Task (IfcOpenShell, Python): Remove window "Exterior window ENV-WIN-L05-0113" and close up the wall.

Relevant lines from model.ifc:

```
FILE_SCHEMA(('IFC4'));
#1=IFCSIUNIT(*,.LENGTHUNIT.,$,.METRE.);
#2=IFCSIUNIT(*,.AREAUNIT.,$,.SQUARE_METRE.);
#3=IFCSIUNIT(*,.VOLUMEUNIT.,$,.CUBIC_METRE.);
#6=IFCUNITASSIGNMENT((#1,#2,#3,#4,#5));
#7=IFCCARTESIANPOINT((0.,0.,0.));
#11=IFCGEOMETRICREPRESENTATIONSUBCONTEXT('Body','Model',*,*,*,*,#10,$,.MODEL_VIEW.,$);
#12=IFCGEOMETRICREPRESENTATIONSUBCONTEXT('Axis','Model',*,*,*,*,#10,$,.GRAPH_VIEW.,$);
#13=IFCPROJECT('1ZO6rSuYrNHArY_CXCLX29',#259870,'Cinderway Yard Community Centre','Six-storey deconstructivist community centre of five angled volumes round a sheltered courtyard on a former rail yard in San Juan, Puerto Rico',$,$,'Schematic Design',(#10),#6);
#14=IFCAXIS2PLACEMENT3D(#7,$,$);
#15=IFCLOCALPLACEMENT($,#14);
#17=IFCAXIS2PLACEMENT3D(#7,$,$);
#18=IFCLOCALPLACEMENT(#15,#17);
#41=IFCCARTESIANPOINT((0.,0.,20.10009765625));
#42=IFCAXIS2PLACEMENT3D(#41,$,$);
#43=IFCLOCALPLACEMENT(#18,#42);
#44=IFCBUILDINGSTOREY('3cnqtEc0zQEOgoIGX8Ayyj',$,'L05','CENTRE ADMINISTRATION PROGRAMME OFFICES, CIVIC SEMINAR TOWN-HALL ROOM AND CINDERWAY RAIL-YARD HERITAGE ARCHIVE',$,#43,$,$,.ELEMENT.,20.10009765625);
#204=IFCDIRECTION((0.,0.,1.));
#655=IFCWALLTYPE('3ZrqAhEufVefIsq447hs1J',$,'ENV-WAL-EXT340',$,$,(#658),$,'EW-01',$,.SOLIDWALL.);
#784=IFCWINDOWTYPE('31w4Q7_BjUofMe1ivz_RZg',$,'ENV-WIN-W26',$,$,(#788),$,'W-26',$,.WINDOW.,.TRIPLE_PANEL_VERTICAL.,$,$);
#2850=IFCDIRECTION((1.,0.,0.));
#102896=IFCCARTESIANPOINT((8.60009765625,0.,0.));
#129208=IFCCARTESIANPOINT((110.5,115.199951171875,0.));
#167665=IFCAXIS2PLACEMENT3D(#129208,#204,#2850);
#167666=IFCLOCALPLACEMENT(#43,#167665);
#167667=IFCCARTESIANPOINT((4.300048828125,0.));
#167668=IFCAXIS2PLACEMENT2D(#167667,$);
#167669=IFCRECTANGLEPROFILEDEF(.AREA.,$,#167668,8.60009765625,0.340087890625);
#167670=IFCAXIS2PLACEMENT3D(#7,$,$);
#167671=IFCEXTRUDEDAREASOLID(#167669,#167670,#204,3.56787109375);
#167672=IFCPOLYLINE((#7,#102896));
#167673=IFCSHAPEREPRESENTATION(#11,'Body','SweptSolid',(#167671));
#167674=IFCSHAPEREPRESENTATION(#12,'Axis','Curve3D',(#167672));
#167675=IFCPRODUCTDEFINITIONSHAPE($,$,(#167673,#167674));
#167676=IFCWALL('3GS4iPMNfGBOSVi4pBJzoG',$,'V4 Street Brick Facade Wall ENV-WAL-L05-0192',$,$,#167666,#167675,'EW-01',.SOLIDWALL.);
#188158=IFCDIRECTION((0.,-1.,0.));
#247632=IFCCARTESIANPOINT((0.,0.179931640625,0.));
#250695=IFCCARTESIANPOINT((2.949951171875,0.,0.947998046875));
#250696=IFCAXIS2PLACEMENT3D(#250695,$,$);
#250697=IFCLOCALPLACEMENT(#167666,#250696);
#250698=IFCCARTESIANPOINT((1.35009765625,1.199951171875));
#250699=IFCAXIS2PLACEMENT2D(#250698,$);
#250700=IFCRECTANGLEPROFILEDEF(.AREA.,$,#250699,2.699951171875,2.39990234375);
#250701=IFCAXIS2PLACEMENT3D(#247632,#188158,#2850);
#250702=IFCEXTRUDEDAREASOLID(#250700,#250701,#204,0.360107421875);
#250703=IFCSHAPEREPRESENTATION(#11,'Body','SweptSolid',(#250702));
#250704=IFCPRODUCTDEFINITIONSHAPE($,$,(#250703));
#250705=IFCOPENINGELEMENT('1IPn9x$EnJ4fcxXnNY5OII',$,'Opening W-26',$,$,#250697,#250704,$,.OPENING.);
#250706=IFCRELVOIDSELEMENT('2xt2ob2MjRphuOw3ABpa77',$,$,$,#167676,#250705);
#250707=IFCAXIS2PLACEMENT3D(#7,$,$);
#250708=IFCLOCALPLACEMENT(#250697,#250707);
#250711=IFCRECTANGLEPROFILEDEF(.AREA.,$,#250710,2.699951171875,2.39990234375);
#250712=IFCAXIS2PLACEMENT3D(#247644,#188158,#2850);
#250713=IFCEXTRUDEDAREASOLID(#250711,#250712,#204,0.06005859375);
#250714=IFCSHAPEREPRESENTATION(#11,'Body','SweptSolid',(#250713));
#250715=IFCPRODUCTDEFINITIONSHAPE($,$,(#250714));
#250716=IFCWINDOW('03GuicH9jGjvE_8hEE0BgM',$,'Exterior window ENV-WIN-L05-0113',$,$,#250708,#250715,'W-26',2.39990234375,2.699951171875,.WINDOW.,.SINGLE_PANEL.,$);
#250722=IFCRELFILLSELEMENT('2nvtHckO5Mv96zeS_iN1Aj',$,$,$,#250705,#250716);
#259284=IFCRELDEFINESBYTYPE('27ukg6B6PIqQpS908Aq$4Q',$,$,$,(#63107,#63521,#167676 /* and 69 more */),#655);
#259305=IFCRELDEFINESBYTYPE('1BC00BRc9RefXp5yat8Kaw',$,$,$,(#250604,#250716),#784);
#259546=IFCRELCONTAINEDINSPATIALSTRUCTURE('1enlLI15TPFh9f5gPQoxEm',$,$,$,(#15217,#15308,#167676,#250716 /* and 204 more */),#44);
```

```python
import ifcopenshell
import ifcopenshell.api.feature
import ifcopenshell.api.root
import ifcopenshell.geom
import ifcopenshell.util.shape

model = ifcopenshell.open("model.ifc")
settings = ifcopenshell.geom.settings()


def volume(element):
    """Net volume in cubic metres, openings subtracted."""
    shape = ifcopenshell.geom.create_shape(settings, element)
    return ifcopenshell.util.shape.get_volume(shape.geometry)


window = model.by_guid("03GuicH9jGjvE_8hEE0BgM")
opening = window.FillsVoids[0].RelatingOpeningElement
wall = opening.VoidsElements[0].RelatingBuildingElement
before = volume(wall)

ifcopenshell.api.root.remove_product(model, product=window)
ifcopenshell.api.feature.remove_feature(model, feature=opening)

after = volume(wall)

print(f"wall volume {before:.3f} -> {after:.3f} m3")

model.write("model_v2.ifc")
```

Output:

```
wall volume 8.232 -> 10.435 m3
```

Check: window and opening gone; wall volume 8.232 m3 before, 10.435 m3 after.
